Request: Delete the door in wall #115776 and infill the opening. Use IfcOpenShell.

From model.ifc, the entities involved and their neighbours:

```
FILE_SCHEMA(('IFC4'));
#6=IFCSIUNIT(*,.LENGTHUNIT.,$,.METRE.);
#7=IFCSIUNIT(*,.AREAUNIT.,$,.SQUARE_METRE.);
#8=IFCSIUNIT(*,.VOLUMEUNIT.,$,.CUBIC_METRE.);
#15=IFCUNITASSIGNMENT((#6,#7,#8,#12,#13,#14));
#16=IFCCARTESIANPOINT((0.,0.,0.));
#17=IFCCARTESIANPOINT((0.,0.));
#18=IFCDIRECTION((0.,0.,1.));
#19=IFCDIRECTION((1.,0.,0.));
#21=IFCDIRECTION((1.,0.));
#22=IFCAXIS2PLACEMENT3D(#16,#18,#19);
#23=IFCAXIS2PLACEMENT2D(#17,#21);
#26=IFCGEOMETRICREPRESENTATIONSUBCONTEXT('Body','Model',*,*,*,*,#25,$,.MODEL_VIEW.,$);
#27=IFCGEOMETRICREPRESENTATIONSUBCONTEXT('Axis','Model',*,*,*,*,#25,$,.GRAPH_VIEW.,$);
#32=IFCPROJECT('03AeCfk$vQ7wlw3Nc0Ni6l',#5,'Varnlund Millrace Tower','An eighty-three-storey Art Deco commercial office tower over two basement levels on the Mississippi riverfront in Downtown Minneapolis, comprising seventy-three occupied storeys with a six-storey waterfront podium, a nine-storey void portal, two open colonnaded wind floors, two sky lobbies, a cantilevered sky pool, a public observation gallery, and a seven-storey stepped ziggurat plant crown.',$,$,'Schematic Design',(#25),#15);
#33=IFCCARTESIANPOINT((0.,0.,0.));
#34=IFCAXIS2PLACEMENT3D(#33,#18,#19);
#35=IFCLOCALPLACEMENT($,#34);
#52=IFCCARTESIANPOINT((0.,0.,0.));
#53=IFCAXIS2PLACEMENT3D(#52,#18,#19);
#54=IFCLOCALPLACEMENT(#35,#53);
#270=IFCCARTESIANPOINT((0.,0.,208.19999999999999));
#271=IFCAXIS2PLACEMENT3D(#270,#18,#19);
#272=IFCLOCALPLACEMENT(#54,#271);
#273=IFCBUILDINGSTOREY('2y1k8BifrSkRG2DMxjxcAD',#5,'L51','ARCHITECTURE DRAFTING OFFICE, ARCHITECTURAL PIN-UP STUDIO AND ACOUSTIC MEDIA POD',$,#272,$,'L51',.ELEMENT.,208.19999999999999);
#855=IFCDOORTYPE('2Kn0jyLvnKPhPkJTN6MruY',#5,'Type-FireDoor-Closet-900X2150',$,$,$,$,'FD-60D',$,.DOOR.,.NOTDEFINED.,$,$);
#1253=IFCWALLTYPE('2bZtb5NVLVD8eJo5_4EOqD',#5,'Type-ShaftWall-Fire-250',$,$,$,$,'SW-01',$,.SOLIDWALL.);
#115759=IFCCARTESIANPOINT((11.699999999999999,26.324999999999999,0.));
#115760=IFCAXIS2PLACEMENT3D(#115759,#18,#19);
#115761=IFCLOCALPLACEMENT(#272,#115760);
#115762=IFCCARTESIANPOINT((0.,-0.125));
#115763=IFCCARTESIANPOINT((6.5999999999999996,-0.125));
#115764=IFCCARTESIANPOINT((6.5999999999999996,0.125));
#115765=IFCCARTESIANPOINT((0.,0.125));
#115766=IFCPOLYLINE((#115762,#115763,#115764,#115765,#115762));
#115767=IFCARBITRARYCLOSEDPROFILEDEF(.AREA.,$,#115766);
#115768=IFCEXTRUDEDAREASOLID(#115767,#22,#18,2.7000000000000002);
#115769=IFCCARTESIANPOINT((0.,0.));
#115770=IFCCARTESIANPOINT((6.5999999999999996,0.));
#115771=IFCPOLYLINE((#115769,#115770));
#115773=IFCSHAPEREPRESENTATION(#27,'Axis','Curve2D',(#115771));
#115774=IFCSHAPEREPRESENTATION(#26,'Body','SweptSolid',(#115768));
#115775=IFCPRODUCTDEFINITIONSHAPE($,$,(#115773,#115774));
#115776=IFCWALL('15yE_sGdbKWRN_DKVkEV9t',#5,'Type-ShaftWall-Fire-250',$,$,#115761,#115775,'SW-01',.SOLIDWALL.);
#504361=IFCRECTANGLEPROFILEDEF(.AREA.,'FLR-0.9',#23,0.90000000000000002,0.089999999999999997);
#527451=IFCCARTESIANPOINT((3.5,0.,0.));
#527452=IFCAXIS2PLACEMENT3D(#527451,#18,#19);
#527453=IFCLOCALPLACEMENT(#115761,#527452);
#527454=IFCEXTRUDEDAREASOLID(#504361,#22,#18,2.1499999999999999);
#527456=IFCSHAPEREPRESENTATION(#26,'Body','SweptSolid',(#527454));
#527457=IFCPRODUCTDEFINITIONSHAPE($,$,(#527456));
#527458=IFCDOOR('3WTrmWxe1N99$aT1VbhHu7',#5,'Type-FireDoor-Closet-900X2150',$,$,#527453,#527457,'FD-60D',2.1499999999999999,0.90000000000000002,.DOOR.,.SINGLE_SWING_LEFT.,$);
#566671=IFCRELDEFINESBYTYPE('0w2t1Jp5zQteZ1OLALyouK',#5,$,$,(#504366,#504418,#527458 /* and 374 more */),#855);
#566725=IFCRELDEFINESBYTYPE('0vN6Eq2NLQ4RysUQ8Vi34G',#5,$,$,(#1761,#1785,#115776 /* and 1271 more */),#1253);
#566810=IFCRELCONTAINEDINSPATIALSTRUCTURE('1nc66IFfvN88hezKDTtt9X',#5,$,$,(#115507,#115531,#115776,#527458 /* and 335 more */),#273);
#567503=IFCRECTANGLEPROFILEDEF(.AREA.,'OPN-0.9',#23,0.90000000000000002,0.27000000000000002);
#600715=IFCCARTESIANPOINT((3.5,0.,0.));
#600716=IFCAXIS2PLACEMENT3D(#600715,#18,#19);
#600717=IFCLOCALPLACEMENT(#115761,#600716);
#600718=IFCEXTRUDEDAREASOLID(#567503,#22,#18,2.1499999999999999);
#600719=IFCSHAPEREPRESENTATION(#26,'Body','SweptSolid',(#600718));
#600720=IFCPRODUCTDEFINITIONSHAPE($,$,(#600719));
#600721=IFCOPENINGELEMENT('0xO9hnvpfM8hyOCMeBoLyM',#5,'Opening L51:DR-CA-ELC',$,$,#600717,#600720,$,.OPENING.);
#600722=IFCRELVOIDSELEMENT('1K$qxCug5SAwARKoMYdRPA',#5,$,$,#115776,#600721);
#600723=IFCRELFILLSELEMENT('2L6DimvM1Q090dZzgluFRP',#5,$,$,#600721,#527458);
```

```python
import ifcopenshell
import ifcopenshell.api.feature
import ifcopenshell.api.root
import ifcopenshell.geom
import ifcopenshell.util.shape

model = ifcopenshell.open("model.ifc")
settings = ifcopenshell.geom.settings()


def volume(element):
    """Net volume in cubic metres, openings subtracted."""
    shape = ifcopenshell.geom.create_shape(settings, element)
    return ifcopenshell.util.shape.get_volume(shape.geometry)


door = model.by_guid("3WTrmWxe1N99$aT1VbhHu7")
opening = door.FillsVoids[0].RelatingOpeningElement
wall = opening.VoidsElements[0].RelatingBuildingElement
before = volume(wall)

ifcopenshell.api.root.remove_product(model, product=door)
ifcopenshell.api.feature.remove_feature(model, feature=opening)

after = volume(wall)

print(f"wall volume {before:.3f} -> {after:.3f} m3")

model.write("model_edited.ifc")
```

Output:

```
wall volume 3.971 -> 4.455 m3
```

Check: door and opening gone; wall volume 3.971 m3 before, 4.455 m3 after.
